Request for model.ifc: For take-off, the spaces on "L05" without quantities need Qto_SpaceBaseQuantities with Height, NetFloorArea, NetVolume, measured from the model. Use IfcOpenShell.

First a look at what the model holds.

```python
import ifcopenshell
import ifcopenshell.util.element
import ifcopenshell.util.unit

model = ifcopenshell.open("model.ifc")
print(model.schema)
for unit_type in ("LENGTHUNIT", "AREAUNIT", "VOLUMEUNIT"):
    print(unit_type, ifcopenshell.util.unit.calculate_unit_scale(model, unit_type))
storey = next(s for s in model.by_type("IfcBuildingStorey") if s.Name == "L05")
spaces = [e for e in ifcopenshell.util.element.get_decomposition(storey) if e.is_a("IfcSpace")]
for e in sorted(spaces, key=lambda e: e.id()):
    print(e.id(), e.is_a(), e.Name, list(ifcopenshell.util.element.get_psets(e, qtos_only=True)), sep=" | ")
```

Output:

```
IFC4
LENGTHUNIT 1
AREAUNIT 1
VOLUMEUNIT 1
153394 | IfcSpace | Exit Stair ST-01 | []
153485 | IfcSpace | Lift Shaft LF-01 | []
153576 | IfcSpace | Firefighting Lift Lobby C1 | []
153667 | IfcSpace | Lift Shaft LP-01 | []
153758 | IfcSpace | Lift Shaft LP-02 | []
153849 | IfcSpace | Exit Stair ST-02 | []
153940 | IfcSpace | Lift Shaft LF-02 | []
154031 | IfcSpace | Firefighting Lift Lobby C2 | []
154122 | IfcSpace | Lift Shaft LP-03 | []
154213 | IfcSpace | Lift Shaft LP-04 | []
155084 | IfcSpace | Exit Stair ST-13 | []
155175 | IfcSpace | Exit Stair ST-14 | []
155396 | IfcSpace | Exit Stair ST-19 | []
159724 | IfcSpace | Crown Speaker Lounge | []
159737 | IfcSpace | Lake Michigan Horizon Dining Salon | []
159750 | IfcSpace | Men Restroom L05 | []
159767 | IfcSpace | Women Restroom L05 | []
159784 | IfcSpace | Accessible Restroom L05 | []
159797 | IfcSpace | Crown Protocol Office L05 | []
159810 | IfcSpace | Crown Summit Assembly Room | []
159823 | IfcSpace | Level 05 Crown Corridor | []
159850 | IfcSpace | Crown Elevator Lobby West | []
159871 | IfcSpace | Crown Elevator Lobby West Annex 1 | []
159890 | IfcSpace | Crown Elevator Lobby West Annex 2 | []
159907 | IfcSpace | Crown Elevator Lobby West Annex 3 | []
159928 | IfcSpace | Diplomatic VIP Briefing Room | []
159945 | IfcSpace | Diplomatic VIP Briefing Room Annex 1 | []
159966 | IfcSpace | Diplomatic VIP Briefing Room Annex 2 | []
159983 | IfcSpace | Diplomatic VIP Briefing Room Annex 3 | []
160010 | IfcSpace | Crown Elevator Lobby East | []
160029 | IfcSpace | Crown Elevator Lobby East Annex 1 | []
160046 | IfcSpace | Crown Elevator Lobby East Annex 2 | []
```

```python
import ifcopenshell
import ifcopenshell.api.pset
import ifcopenshell.geom
import ifcopenshell.util.element
import ifcopenshell.util.shape
import ifcopenshell.util.unit

model = ifcopenshell.open("model.ifc")
unit_scale = ifcopenshell.util.unit.calculate_unit_scale(model)
area_scale = ifcopenshell.util.unit.calculate_unit_scale(model, "AREAUNIT")
volume_scale = ifcopenshell.util.unit.calculate_unit_scale(model, "VOLUMEUNIT")
settings = ifcopenshell.geom.settings()

storey = next(s for s in model.by_type("IfcBuildingStorey") if s.Name == "L05")
spaces = [e for e in ifcopenshell.util.element.get_decomposition(storey) if e.is_a("IfcSpace")]

for e in sorted(spaces, key=lambda e: e.id()):
    if ifcopenshell.util.element.get_psets(e, qtos_only=True, should_inherit=False):
        continue
    # Geometry comes back in metres, in the element's own axes.
    shape = ifcopenshell.geom.create_shape(settings, e)
    values = {
        "Height": ifcopenshell.util.shape.get_z(shape.geometry) / unit_scale,
        "NetFloorArea": ifcopenshell.util.shape.get_footprint_area(shape.geometry) / area_scale,
        "NetVolume": ifcopenshell.util.shape.get_volume(shape.geometry) / volume_scale,
    }
    qto = ifcopenshell.api.pset.add_qto(model, product=e, name="Qto_SpaceBaseQuantities")
    ifcopenshell.api.pset.edit_qto(model, qto=qto, properties=values)
    print(e.id(), {k: round(v, 3) for k, v in values.items()})

model.write("model_edited.ifc")
```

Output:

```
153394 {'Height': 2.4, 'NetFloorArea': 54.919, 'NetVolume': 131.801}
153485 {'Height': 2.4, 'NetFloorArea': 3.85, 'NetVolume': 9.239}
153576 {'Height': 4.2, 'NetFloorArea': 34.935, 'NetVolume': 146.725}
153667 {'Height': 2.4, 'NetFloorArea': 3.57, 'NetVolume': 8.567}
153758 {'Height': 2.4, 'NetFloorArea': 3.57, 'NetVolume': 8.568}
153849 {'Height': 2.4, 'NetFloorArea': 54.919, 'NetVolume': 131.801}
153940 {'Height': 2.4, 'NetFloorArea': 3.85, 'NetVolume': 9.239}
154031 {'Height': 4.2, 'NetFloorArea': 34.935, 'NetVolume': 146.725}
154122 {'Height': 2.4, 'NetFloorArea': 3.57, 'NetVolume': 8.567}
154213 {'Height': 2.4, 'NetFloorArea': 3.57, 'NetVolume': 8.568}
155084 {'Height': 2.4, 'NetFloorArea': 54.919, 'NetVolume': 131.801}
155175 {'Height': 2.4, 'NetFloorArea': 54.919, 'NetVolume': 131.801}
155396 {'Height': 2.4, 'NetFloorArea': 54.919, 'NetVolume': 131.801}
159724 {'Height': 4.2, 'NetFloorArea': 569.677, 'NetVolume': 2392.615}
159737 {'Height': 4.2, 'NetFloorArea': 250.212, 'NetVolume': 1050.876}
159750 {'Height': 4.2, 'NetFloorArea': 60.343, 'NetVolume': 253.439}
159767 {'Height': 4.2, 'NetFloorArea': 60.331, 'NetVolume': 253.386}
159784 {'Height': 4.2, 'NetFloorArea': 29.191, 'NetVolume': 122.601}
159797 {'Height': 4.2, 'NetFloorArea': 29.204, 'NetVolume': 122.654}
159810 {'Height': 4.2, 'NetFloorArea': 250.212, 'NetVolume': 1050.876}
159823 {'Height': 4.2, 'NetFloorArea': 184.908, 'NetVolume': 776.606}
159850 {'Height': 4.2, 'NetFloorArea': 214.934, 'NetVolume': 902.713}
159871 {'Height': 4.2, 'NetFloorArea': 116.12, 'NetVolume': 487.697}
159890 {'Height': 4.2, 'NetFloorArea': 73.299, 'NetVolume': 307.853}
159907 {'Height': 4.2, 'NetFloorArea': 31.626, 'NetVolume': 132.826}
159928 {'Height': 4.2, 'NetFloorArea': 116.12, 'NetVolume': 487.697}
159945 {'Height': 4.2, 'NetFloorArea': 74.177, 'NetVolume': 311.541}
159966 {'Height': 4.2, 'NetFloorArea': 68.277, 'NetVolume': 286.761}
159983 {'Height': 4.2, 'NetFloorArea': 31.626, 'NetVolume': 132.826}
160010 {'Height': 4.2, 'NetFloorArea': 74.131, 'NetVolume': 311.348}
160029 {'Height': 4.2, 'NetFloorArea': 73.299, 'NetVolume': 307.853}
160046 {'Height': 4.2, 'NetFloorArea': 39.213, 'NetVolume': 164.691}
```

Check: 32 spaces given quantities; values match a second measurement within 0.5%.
